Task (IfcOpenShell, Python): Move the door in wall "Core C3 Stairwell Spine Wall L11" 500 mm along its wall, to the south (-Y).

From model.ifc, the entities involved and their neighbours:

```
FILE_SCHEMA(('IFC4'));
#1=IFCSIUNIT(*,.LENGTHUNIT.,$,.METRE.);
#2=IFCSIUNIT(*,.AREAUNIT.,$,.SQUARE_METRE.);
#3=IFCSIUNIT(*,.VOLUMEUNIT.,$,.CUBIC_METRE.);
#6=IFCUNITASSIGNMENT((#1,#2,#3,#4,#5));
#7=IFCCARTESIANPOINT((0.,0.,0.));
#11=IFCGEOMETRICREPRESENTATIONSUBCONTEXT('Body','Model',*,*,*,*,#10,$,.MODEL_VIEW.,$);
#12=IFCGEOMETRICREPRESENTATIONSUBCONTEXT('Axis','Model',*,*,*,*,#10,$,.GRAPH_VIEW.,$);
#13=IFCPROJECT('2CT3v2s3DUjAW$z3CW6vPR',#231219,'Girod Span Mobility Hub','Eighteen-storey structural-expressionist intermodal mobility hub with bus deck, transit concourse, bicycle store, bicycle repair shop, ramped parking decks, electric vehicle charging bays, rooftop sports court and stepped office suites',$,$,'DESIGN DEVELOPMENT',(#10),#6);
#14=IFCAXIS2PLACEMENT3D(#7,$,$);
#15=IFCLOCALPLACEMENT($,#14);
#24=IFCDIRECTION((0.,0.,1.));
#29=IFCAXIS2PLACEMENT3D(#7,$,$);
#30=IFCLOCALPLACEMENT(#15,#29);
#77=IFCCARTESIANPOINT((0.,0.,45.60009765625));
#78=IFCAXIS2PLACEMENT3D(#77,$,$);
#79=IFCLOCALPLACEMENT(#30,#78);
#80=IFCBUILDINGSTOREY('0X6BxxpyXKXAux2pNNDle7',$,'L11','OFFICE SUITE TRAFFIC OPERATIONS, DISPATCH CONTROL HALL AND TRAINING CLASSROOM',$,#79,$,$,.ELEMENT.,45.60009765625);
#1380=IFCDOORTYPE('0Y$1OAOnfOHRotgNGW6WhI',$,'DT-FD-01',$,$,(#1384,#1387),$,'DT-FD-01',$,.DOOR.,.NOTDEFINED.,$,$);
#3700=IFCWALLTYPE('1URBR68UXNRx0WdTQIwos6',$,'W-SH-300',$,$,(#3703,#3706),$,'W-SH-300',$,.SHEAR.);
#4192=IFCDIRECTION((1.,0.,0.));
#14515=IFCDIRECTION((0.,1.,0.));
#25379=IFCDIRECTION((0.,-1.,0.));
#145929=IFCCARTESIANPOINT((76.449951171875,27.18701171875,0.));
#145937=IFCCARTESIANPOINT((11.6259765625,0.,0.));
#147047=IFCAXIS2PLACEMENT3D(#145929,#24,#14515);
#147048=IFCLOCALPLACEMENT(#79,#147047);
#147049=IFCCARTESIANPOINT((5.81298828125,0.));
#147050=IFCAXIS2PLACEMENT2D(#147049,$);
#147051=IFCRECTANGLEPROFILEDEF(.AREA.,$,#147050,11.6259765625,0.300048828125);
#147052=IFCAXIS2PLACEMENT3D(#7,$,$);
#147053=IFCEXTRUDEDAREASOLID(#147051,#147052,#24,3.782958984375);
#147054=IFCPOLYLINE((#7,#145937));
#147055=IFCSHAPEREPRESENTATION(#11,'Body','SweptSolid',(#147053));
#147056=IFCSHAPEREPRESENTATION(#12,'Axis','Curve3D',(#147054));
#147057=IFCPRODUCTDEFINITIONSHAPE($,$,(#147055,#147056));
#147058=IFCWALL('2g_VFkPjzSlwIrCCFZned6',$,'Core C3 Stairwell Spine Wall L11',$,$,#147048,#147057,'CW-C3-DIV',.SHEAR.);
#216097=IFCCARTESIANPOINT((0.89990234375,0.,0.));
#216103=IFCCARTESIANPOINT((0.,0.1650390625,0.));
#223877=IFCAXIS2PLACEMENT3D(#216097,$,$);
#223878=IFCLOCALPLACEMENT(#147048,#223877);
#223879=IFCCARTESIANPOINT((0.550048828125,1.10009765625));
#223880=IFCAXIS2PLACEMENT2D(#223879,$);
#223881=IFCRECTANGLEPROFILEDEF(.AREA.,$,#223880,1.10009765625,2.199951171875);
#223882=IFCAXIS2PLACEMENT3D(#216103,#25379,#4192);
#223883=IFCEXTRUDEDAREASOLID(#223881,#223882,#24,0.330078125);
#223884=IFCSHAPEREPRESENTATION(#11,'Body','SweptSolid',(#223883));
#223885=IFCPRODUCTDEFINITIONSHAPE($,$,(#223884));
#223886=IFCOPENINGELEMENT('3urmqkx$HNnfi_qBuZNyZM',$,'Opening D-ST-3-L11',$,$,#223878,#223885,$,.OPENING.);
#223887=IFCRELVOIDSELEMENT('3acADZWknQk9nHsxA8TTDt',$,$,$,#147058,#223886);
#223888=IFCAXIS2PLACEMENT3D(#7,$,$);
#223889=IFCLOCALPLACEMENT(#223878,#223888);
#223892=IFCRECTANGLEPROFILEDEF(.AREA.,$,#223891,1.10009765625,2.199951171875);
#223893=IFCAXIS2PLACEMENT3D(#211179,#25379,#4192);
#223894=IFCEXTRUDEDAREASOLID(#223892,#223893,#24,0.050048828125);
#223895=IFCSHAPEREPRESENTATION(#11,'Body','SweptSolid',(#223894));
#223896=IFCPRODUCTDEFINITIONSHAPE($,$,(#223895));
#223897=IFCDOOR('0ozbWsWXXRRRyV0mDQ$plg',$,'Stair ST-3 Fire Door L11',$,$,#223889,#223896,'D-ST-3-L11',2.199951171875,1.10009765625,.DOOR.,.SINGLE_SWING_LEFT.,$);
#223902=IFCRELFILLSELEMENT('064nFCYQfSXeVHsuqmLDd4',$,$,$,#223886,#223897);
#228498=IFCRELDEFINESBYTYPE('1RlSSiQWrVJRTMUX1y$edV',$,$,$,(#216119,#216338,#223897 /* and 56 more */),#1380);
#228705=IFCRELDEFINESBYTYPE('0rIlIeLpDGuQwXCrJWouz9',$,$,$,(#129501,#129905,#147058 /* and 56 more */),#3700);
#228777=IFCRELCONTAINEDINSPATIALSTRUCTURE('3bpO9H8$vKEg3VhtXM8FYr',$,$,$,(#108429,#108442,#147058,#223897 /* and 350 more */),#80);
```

```python
import ifcopenshell
import ifcopenshell.api.geometry
import ifcopenshell.util.placement

model = ifcopenshell.open("model.ifc")

door = model.by_guid("0ozbWsWXXRRRyV0mDQ$plg")
opening = door.FillsVoids[0].RelatingOpeningElement
wall = opening.VoidsElements[0].RelatingBuildingElement

wall_matrix = ifcopenshell.util.placement.get_local_placement(wall.ObjectPlacement)
shift = wall_matrix[:3, 0] * -0.5
before = ifcopenshell.util.placement.get_local_placement(door.ObjectPlacement)[:3, 3].copy()

# The door is placed relative to its opening, so it follows when the opening moves.
matrix = ifcopenshell.util.placement.get_local_placement(opening.ObjectPlacement)
matrix[:3, 3] += shift
ifcopenshell.api.geometry.edit_object_placement(
    model, product=opening, matrix=matrix, is_si=False, should_transform_children=True
)

after = ifcopenshell.util.placement.get_local_placement(door.ObjectPlacement)[:3, 3]
print("door moved by", (after - before).round(3) + 0.0)

model.write("model_v2.ifc")
```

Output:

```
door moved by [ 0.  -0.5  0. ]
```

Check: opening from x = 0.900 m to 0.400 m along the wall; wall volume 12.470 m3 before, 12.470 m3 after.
